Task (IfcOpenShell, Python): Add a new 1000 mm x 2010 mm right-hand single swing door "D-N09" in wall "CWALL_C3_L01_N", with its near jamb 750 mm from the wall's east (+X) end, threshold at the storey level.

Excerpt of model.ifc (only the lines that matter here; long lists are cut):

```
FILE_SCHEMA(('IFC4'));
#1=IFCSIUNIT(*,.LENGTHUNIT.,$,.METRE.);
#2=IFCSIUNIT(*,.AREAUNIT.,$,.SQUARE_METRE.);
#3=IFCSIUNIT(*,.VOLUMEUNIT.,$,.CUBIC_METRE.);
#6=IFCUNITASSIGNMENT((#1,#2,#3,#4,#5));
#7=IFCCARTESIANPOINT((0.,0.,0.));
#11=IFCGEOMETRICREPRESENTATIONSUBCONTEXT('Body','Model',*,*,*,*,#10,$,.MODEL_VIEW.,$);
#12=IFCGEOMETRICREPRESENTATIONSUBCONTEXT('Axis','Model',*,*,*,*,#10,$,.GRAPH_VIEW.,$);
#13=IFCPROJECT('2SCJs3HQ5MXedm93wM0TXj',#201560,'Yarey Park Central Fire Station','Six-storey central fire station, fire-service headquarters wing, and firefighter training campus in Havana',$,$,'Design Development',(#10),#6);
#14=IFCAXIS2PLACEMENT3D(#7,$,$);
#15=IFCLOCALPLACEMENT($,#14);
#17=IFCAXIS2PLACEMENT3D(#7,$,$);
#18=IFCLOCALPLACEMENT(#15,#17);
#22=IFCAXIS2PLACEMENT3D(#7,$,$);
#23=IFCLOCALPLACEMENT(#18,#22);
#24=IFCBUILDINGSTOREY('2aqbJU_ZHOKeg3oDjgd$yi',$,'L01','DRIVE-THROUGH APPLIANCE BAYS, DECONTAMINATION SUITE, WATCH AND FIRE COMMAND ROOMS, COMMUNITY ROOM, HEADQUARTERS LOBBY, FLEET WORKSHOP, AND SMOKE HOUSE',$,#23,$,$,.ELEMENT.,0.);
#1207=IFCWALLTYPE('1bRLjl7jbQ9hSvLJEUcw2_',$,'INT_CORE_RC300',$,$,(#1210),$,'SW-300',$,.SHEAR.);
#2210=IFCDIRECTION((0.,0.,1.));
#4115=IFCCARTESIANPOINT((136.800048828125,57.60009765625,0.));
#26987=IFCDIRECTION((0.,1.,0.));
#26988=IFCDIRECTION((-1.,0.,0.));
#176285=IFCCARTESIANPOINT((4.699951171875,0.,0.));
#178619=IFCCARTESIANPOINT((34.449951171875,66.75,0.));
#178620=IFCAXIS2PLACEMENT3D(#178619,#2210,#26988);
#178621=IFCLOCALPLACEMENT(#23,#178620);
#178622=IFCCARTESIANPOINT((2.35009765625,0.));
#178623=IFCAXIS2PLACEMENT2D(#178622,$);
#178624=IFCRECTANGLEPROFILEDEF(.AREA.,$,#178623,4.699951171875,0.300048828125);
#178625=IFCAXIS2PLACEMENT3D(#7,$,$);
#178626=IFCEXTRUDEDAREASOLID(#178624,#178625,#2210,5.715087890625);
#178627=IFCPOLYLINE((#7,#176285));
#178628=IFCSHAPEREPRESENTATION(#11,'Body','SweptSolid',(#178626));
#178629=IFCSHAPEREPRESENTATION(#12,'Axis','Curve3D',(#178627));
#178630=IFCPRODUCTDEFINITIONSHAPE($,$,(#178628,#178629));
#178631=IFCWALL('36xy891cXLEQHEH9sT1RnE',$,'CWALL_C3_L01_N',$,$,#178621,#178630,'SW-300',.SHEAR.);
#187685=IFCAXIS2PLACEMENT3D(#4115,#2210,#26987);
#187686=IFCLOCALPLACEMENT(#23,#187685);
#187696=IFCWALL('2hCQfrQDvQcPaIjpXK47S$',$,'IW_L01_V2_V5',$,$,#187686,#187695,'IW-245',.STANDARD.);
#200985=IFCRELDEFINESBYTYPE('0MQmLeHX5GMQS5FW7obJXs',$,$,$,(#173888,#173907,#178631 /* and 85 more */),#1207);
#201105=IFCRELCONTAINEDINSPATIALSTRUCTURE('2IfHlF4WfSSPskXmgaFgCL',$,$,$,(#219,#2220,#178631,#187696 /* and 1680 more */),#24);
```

```python
import numpy as np
import ifcopenshell
import ifcopenshell.api.feature
import ifcopenshell.api.geometry
import ifcopenshell.api.root
import ifcopenshell.api.spatial
import ifcopenshell.geom
import ifcopenshell.util.element
import ifcopenshell.util.placement
import ifcopenshell.util.representation
import ifcopenshell.util.shape
import ifcopenshell.util.unit

model = ifcopenshell.open("model.ifc")
unit_scale = ifcopenshell.util.unit.calculate_unit_scale(model)
settings = ifcopenshell.geom.settings()


def volume(element):
    """Net volume in cubic metres, openings subtracted."""
    shape = ifcopenshell.geom.create_shape(settings, element)
    return ifcopenshell.util.shape.get_volume(shape.geometry)


wall = model.by_id(178631)
storey = ifcopenshell.util.element.get_container(wall, ifc_class="IfcBuildingStorey")
context = ifcopenshell.util.representation.get_context(model, "Model", "Body", "MODEL_VIEW")
before = volume(wall)

width, height, from_end, sill = 1, 2.01, 0.75, 0.0  # metres

# The wall runs along its own X axis, and the end named is its -X end.
wall_shape = ifcopenshell.geom.create_shape(settings, wall)
x, y, z = ifcopenshell.util.shape.get_vertices(wall_shape.geometry).T
start = x.min() + from_end
face, thickness = float(y.min()), float(y.max() - y.min())
wall_matrix = ifcopenshell.util.placement.get_local_placement(wall.ObjectPlacement)
level = ifcopenshell.util.placement.get_local_placement(storey.ObjectPlacement)[2, 3]


def in_wall(x, y):
    """Placement at x, y metres in the wall's axes, at sill height."""
    matrix = wall_matrix.copy()
    matrix[:, 3] = wall_matrix @ np.array([x / unit_scale, y / unit_scale, 0.0, 1.0])
    matrix[2, 3] = level + sill / unit_scale
    return matrix


# Opening: a box that overshoots both wall faces by 50 mm.
opening = ifcopenshell.api.root.create_entity(model, ifc_class="IfcOpeningElement", predefined_type="OPENING")
box = ifcopenshell.api.geometry.add_wall_representation(
    model, context=context, length=width, height=height, thickness=thickness + 0.1
)
ifcopenshell.api.geometry.assign_representation(model, product=opening, representation=box)
ifcopenshell.api.geometry.edit_object_placement(model, product=opening, matrix=in_wall(start, face - 0.05), is_si=False)
ifcopenshell.api.feature.add_feature(model, feature=opening, element=wall)

door = ifcopenshell.api.root.create_entity(model, ifc_class="IfcDoor", name="D-N09", predefined_type="DOOR")
door.OverallWidth, door.OverallHeight = width / unit_scale, height / unit_scale
door.OperationType = "SINGLE_SWING_RIGHT"
body = ifcopenshell.api.geometry.add_door_representation(
    model,
    context=context,
    overall_width=door.OverallWidth,
    overall_height=door.OverallHeight,
    operation_type="SINGLE_SWING_RIGHT",
    lining_properties={"LiningDepth": thickness / unit_scale, "ThresholdDepth": thickness / unit_scale},
)
ifcopenshell.api.geometry.assign_representation(model, product=door, representation=body)
ifcopenshell.api.spatial.assign_container(model, products=[door], relating_structure=storey)
ifcopenshell.api.feature.add_filling(model, opening=opening, element=door)

# The lining spans the wall, so the door starts at the wall face.
ifcopenshell.api.geometry.edit_object_placement(model, product=door, matrix=in_wall(start, face), is_si=False)

after = volume(wall)

print(f"wall volume {before:.3f} -> {after:.3f} m3")

model.write("model-out.ifc")
```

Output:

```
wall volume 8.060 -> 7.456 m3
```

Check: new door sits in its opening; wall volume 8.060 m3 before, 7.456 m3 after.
